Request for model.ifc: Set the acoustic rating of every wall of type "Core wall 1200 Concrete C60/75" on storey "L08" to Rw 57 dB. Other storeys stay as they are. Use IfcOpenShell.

First a look at what the model holds.

```python
import ifcopenshell
import ifcopenshell.util.element

model = ifcopenshell.open("model.ifc")
print(model.schema)
storey = next(s for s in model.by_type("IfcBuildingStorey") if s.Name == "L08")
walls = [e for e in ifcopenshell.util.element.get_decomposition(storey) if e.is_a("IfcWall")]
seen = {}
for e in walls:
    element_type = ifcopenshell.util.element.get_type(e)
    key = (element_type.Name if element_type != e and element_type else None, ifcopenshell.util.element.get_pset(e, "Pset_WallCommon", "AcousticRating"))
    seen[key] = seen.get(key, 0) + 1
for (name, value), count in sorted(seen.items(), key=str):
    print(count, "x", name, "|", value)
```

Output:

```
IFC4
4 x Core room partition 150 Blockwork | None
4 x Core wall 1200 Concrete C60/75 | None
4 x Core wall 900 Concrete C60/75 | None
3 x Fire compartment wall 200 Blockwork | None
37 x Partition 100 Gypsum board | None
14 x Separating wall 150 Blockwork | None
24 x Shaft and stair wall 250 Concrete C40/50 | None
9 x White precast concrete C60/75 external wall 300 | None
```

```python
import ifcopenshell
import ifcopenshell.api.pset
import ifcopenshell.util.element

model = ifcopenshell.open("model.ifc")

storey = next(s for s in model.by_type("IfcBuildingStorey") if s.Name == "L08")
walls = [e for e in ifcopenshell.util.element.get_decomposition(storey) if e.is_a("IfcWall")]

count = 0
for e in walls:
    element_type = ifcopenshell.util.element.get_type(e)
    if element_type in (None, e) or element_type.Name != "Core wall 1200 Concrete C60/75":
        continue
    found = ifcopenshell.util.element.get_pset(e, "Pset_WallCommon", should_inherit=False)
    if found:
        pset = model.by_id(found["id"])
        if len(ifcopenshell.util.element.get_elements_by_pset(pset)) > 1:
            pset = ifcopenshell.api.pset.unshare_pset(model, products=[e], pset=pset)[0]
    else:
        pset = ifcopenshell.api.pset.add_pset(model, product=e, name="Pset_WallCommon")
    ifcopenshell.api.pset.edit_pset(model, pset=pset, properties={"AcousticRating": "Rw 57 dB"})
    count += 1

print(count, "walls updated")

model.write("model-out.ifc")
```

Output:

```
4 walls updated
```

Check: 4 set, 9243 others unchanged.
